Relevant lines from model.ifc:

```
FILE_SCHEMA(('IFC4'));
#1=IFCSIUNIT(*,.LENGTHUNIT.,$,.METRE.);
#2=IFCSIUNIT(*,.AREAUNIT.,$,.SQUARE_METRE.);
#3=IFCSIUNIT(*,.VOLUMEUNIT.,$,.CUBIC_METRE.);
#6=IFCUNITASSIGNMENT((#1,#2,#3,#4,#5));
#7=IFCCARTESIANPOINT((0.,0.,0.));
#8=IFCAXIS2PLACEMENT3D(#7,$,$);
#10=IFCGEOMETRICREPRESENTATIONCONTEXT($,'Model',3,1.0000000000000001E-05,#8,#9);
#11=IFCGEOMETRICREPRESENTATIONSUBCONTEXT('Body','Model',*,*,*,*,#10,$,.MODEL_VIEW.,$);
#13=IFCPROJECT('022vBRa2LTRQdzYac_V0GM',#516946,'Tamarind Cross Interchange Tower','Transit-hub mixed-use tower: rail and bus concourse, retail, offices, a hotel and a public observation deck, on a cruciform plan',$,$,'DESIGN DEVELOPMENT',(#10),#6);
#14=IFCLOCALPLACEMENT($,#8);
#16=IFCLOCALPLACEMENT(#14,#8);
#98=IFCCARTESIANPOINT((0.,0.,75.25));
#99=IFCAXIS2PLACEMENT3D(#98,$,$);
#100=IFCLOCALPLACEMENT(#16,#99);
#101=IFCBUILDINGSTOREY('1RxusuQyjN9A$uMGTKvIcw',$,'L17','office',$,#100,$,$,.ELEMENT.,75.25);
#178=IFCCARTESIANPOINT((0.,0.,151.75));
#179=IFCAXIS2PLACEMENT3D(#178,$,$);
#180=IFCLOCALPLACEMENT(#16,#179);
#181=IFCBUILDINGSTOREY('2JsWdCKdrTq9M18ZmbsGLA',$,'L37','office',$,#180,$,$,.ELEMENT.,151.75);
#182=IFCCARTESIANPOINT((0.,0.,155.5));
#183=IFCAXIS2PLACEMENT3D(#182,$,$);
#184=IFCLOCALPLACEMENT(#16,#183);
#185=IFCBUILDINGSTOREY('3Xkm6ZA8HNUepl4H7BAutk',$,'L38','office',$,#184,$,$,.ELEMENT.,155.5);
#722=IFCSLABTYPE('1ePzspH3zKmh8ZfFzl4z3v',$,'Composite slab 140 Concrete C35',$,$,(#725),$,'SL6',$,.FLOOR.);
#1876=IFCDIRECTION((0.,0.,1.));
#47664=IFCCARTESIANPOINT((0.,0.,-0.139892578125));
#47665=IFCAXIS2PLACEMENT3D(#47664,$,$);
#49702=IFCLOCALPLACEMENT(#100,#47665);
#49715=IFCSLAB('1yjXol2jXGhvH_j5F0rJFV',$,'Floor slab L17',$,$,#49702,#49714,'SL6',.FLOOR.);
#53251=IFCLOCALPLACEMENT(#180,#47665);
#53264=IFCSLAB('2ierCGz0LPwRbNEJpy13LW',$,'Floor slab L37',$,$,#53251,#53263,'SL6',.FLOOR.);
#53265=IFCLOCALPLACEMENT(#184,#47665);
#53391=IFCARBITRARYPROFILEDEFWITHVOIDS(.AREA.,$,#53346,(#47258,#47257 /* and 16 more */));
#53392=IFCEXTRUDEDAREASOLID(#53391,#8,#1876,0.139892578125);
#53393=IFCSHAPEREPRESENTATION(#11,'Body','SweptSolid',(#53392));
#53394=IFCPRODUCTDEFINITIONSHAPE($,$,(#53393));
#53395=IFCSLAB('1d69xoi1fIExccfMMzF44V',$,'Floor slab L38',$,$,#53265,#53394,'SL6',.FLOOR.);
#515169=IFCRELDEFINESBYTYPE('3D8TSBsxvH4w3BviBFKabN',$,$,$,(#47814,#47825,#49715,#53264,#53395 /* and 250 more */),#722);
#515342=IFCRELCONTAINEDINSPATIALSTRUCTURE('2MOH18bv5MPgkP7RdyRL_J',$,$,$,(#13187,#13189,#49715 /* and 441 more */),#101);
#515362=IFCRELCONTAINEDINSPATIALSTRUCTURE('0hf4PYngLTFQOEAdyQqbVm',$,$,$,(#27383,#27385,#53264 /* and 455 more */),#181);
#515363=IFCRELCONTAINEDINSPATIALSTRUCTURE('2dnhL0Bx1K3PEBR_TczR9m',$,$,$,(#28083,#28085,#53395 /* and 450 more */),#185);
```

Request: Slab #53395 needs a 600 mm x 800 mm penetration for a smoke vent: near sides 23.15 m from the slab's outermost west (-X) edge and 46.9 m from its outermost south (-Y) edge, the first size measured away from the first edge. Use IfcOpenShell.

```python
import numpy as np
import ifcopenshell
import ifcopenshell.api.feature
import ifcopenshell.api.geometry
import ifcopenshell.api.root
import ifcopenshell.geom
import ifcopenshell.util.placement
import ifcopenshell.util.representation
import ifcopenshell.util.shape
import ifcopenshell.util.unit

model = ifcopenshell.open("model.ifc")
unit_scale = ifcopenshell.util.unit.calculate_unit_scale(model)
settings = ifcopenshell.geom.settings()


def volume(element):
    """Net volume in cubic metres, openings subtracted."""
    shape = ifcopenshell.geom.create_shape(settings, element)
    return ifcopenshell.util.shape.get_volume(shape.geometry)


slab = model.by_guid("1d69xoi1fIExccfMMzF44V")
before = volume(slab)

# Extent in the slab's own axes, in metres. The edges named are its -X and -Y sides.
slab_shape = ifcopenshell.geom.create_shape(settings, slab)
vertices = ifcopenshell.util.shape.get_vertices(slab_shape.geometry)
x_min, y_min, bottom = vertices.min(axis=0)
top = vertices[:, 2].max()

opening = ifcopenshell.api.root.create_entity(model, ifc_class="IfcOpeningElement", name="Smoke vent opening", predefined_type="OPENING")
context = ifcopenshell.util.representation.get_context(model, "Model", "Body", "MODEL_VIEW")
width, depth = 0.6, 0.8
outline = [(0.0, 0.0), (width, 0.0), (width, depth), (0.0, depth), (0.0, 0.0)]
# Overshoot both faces by 50 mm so the cut is clean.
shape = ifcopenshell.api.geometry.add_slab_representation(
    model, context=context, depth=top - bottom + 0.1, polyline=outline
)
ifcopenshell.api.geometry.assign_representation(model, product=opening, representation=shape)

matrix = ifcopenshell.util.placement.get_local_placement(slab.ObjectPlacement)
matrix[:, 3] = matrix @ np.append(np.array([x_min + 23.15, y_min + 46.9, bottom - 0.05]) / unit_scale, 1.0)
ifcopenshell.api.geometry.edit_object_placement(model, product=opening, matrix=matrix, is_si=False)
ifcopenshell.api.feature.add_feature(model, feature=opening, element=slab)

after = volume(slab)

print(f"slab volume {before:.3f} -> {after:.3f} m3")

model.write("model_updated.ifc")
```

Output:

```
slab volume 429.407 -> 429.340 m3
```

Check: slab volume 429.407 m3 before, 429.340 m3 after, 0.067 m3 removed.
